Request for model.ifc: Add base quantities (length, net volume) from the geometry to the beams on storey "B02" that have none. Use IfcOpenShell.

First a look at what the model holds.

```python
import ifcopenshell
import ifcopenshell.util.element
import ifcopenshell.util.unit

model = ifcopenshell.open("model.ifc")
print(model.schema)
for unit_type in ("LENGTHUNIT", "AREAUNIT", "VOLUMEUNIT"):
    print(unit_type, ifcopenshell.util.unit.calculate_unit_scale(model, unit_type))
storey = next(s for s in model.by_type("IfcBuildingStorey") if s.Name == "B02")
beams = [e for e in ifcopenshell.util.element.get_decomposition(storey) if e.is_a("IfcBeam")]
for e in sorted(beams, key=lambda e: e.id()):
    print(e.id(), e.is_a(), e.Name, list(ifcopenshell.util.element.get_psets(e, qtos_only=True)), sep=" | ")
```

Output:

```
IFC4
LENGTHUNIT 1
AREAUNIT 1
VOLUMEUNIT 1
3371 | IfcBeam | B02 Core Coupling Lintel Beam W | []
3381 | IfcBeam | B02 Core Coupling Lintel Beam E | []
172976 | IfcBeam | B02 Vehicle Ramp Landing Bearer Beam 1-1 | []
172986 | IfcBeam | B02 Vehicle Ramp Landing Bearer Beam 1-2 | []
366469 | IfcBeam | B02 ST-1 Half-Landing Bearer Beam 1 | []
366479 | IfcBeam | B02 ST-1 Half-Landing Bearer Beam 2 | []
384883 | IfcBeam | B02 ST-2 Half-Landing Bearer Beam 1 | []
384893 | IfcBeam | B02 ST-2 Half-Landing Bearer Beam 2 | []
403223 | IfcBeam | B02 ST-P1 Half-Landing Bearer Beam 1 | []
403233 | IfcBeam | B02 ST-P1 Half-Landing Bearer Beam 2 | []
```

```python
import ifcopenshell
import ifcopenshell.api.pset
import ifcopenshell.geom
import ifcopenshell.util.element
import ifcopenshell.util.shape
import ifcopenshell.util.unit

model = ifcopenshell.open("model.ifc")
unit_scale = ifcopenshell.util.unit.calculate_unit_scale(model)
volume_scale = ifcopenshell.util.unit.calculate_unit_scale(model, "VOLUMEUNIT")
settings = ifcopenshell.geom.settings()

storey = next(s for s in model.by_type("IfcBuildingStorey") if s.Name == "B02")
beams = [e for e in ifcopenshell.util.element.get_decomposition(storey) if e.is_a("IfcBeam")]

for e in sorted(beams, key=lambda e: e.id()):
    if ifcopenshell.util.element.get_psets(e, qtos_only=True, should_inherit=False):
        continue
    # Geometry comes back in metres, in the element's own axes.
    shape = ifcopenshell.geom.create_shape(settings, e)
    values = {
        "Length": ifcopenshell.util.shape.get_max_xyz(shape.geometry) / unit_scale,
        "NetVolume": ifcopenshell.util.shape.get_volume(shape.geometry) / volume_scale,
    }
    qto = ifcopenshell.api.pset.add_qto(model, product=e, name="Qto_BeamBaseQuantities")
    ifcopenshell.api.pset.edit_qto(model, qto=qto, properties=values)
    print(e.id(), {k: round(v, 3) for k, v in values.items()})

model.write("model_updated.ifc")
```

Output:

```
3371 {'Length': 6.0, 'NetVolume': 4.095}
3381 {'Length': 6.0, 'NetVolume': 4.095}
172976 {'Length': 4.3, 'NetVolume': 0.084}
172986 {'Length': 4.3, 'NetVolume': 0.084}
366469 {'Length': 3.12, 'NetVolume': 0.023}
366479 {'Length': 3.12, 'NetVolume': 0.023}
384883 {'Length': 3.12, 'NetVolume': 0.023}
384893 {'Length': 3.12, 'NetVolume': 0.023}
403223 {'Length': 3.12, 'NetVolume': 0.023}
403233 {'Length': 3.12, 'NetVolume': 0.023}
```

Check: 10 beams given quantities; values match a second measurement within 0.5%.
